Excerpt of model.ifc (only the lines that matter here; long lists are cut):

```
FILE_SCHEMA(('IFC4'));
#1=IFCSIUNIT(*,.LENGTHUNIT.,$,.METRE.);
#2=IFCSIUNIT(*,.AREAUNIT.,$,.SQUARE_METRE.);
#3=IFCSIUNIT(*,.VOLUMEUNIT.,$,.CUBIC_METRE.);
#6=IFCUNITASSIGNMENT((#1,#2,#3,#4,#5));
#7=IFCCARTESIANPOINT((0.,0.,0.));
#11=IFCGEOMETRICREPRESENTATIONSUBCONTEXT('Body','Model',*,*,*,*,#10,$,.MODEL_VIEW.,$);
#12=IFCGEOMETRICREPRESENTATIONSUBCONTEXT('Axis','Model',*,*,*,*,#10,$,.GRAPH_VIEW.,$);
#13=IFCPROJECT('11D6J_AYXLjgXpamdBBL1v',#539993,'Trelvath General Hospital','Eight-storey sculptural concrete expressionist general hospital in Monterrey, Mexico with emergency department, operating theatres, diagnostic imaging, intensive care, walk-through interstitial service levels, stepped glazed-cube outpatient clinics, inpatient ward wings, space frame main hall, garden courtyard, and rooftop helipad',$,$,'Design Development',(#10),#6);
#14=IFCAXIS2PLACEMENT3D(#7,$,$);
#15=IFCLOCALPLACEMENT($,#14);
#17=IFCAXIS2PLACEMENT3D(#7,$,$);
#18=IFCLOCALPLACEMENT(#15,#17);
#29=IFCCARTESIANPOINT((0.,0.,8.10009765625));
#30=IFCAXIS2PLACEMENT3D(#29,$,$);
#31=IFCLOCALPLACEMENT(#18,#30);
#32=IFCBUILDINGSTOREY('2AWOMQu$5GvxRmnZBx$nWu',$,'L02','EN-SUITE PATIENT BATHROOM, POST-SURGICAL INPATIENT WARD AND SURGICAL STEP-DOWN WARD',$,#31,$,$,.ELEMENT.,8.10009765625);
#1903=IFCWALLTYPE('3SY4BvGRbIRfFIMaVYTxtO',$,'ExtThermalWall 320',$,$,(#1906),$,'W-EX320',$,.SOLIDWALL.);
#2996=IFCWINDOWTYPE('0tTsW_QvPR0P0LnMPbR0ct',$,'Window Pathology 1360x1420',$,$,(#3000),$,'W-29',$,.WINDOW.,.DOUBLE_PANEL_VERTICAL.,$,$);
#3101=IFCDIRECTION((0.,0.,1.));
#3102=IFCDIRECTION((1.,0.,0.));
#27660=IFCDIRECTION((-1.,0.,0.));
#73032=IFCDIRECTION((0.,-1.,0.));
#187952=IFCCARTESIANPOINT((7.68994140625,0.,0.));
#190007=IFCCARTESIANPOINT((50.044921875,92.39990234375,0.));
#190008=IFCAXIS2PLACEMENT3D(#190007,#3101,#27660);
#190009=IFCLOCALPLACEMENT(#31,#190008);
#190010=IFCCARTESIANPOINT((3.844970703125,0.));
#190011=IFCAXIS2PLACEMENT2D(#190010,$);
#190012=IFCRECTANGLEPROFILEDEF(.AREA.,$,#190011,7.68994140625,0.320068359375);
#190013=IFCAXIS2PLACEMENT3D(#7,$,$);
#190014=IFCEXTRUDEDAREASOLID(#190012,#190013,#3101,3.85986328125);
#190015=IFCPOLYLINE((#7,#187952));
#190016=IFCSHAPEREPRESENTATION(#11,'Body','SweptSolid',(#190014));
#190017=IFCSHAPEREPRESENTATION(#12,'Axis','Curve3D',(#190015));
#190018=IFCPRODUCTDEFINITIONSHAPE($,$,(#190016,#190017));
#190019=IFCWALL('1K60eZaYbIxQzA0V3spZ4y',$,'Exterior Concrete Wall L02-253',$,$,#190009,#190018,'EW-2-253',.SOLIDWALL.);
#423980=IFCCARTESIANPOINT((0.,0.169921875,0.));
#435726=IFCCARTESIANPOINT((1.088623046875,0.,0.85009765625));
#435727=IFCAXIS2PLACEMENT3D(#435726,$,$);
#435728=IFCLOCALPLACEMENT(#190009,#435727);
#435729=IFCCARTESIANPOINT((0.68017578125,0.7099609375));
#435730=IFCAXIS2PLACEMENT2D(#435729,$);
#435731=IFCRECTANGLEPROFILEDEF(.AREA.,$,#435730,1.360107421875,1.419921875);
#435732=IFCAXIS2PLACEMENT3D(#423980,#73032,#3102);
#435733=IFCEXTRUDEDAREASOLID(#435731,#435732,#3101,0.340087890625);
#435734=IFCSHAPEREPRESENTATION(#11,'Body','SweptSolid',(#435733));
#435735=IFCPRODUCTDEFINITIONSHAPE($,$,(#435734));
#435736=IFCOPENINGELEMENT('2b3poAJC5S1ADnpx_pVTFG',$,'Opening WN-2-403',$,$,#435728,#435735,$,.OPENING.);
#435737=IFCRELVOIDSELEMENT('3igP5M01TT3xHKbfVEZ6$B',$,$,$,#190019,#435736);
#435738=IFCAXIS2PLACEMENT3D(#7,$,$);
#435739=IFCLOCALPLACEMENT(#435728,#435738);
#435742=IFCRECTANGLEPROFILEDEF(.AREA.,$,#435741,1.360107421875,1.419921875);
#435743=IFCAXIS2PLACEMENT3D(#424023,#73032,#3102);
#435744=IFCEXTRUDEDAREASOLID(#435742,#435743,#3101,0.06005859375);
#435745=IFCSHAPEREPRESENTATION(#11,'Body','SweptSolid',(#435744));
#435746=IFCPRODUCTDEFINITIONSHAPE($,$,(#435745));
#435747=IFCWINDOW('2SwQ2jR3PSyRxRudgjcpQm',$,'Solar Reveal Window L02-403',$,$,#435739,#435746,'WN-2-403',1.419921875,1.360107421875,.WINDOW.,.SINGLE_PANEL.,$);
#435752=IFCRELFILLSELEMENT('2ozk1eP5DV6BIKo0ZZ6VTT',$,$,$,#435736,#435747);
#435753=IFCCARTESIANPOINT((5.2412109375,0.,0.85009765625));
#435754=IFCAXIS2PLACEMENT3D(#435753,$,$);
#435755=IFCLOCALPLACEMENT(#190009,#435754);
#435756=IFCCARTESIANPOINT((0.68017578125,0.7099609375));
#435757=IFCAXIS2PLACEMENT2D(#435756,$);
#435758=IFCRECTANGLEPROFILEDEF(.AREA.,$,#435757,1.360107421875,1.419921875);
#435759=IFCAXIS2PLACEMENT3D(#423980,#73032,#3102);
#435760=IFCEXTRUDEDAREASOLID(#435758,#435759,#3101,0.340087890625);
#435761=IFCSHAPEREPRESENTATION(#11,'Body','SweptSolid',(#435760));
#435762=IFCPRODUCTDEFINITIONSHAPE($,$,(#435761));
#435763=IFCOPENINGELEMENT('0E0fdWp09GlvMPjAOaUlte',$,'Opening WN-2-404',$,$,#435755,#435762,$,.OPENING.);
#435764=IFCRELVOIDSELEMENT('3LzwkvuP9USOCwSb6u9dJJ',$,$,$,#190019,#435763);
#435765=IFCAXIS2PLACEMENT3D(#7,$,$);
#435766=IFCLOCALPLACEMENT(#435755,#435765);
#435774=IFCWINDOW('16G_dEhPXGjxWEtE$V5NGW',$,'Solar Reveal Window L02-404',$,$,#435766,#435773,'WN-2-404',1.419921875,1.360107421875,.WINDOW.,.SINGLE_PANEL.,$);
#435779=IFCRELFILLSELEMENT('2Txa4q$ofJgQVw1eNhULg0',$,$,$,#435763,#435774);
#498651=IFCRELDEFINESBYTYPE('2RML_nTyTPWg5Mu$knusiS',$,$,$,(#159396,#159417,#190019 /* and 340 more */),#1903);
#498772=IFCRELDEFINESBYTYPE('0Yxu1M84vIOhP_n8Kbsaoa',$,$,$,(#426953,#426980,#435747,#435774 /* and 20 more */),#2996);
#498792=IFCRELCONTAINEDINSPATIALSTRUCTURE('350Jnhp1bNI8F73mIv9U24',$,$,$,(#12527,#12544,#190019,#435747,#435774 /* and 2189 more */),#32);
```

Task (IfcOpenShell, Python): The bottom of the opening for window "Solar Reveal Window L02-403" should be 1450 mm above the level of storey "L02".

```python
import numpy as np
import ifcopenshell
import ifcopenshell.api.geometry
import ifcopenshell.geom
import ifcopenshell.util.element
import ifcopenshell.util.placement
import ifcopenshell.util.shape
import ifcopenshell.util.unit

model = ifcopenshell.open("model.ifc")
unit_scale = ifcopenshell.util.unit.calculate_unit_scale(model)

window = model.by_id(435747)
opening = window.FillsVoids[0].RelatingOpeningElement
storey = ifcopenshell.util.element.get_container(window, ifc_class="IfcBuildingStorey")
level = ifcopenshell.util.placement.get_local_placement(storey.ObjectPlacement)[2, 3]

# The opening's origin need not be at the sill, so measure its lowest point.
shape = ifcopenshell.geom.create_shape(ifcopenshell.geom.settings(), opening)
bottom = ifcopenshell.util.shape.get_shape_bottom_elevation(shape, shape.geometry) / unit_scale
dz = level + 1.45 / unit_scale - bottom

shift = np.array([0.0, 0.0, dz])
# The window is placed relative to its opening, so it follows when the opening moves.
matrix = ifcopenshell.util.placement.get_local_placement(opening.ObjectPlacement)
matrix[:3, 3] += shift
ifcopenshell.api.geometry.edit_object_placement(
    model, product=opening, matrix=matrix, is_si=False, should_transform_children=True
)

print(f"moved by {dz * unit_scale:+.3f} m")

model.write("model_updated.ifc")
```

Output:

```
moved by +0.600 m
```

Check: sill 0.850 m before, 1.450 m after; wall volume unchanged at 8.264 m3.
